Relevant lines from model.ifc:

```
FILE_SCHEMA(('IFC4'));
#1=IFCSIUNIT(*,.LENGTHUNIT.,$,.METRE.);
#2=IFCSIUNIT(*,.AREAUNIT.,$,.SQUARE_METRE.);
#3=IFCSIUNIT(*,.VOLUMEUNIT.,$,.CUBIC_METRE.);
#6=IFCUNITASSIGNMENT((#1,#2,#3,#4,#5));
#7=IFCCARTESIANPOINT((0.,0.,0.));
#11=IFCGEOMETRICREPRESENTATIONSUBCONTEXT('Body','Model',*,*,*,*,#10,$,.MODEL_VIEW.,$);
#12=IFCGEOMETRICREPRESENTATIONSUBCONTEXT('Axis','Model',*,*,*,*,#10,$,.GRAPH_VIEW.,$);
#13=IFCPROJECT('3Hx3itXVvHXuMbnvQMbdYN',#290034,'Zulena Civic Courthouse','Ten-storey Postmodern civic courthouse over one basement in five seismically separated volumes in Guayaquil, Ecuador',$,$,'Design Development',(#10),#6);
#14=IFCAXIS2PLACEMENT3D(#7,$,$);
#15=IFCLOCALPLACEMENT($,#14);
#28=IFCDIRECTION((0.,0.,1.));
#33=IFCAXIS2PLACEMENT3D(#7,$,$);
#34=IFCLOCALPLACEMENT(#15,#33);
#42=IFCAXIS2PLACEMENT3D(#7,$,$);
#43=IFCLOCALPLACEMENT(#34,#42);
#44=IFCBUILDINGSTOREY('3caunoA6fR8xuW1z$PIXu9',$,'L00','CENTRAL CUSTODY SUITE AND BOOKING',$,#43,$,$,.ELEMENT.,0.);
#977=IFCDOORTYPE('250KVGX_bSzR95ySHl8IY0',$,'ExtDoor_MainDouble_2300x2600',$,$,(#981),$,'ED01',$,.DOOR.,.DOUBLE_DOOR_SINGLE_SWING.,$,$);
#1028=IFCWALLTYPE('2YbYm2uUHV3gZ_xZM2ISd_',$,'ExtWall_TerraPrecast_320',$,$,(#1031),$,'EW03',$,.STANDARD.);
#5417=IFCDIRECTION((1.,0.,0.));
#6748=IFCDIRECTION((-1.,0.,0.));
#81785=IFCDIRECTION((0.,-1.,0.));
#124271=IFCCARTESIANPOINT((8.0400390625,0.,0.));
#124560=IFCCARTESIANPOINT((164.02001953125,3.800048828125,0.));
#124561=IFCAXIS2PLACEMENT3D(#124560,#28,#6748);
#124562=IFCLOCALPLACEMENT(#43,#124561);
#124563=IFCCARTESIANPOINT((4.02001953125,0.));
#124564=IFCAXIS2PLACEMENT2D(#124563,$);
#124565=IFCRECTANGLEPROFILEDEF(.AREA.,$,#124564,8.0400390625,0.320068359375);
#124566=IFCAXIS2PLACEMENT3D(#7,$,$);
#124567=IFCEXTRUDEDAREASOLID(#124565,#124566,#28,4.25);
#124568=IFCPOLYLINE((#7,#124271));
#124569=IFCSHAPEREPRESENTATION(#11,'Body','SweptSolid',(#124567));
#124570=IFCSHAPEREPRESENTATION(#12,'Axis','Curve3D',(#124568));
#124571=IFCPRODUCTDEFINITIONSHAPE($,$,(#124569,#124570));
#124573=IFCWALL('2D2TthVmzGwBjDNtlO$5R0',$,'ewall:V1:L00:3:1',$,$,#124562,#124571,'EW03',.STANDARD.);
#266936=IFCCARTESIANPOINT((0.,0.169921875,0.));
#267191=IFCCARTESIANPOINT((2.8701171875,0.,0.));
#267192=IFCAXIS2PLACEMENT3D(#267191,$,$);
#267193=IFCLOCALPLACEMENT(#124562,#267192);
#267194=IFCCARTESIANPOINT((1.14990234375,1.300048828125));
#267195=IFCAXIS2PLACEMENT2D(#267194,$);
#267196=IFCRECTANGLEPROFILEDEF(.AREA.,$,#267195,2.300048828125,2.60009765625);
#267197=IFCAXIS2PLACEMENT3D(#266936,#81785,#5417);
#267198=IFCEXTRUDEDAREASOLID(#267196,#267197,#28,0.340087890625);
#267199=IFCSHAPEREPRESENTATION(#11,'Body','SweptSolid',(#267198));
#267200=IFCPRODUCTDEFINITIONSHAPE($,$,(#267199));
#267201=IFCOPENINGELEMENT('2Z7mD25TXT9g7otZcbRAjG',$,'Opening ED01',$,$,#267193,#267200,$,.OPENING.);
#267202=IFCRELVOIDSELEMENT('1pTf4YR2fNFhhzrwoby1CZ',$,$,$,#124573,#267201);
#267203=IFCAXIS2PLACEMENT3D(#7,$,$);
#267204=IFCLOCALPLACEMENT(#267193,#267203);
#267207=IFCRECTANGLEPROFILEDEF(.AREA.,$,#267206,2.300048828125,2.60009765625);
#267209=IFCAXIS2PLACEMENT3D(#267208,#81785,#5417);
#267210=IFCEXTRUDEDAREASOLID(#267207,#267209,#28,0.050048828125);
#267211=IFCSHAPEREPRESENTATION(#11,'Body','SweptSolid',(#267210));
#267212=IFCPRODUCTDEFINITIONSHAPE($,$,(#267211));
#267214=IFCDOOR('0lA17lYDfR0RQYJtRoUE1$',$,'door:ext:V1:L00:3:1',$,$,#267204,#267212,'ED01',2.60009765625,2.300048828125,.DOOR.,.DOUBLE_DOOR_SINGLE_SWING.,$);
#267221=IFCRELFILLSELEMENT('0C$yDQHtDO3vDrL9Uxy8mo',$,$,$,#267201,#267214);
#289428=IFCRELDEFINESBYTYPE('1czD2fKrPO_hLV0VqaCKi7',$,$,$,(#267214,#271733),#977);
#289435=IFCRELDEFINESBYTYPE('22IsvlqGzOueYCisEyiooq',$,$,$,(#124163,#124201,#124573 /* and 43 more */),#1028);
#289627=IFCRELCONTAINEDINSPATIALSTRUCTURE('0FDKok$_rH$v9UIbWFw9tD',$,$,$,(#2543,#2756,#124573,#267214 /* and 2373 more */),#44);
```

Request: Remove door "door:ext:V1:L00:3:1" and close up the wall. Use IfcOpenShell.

```python
import ifcopenshell
import ifcopenshell.api.feature
import ifcopenshell.api.root
import ifcopenshell.geom
import ifcopenshell.util.shape

model = ifcopenshell.open("model.ifc")
settings = ifcopenshell.geom.settings()


def volume(element):
    """Net volume in cubic metres, openings subtracted."""
    shape = ifcopenshell.geom.create_shape(settings, element)
    return ifcopenshell.util.shape.get_volume(shape.geometry)


door = model.by_guid("0lA17lYDfR0RQYJtRoUE1$")
opening = door.FillsVoids[0].RelatingOpeningElement
wall = opening.VoidsElements[0].RelatingBuildingElement
before = volume(wall)

ifcopenshell.api.root.remove_product(model, product=door)
ifcopenshell.api.feature.remove_feature(model, feature=opening)

after = volume(wall)

print(f"wall volume {before:.3f} -> {after:.3f} m3")

model.write("model_rev.ifc")
```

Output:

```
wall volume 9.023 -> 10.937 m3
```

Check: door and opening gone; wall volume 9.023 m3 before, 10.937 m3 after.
